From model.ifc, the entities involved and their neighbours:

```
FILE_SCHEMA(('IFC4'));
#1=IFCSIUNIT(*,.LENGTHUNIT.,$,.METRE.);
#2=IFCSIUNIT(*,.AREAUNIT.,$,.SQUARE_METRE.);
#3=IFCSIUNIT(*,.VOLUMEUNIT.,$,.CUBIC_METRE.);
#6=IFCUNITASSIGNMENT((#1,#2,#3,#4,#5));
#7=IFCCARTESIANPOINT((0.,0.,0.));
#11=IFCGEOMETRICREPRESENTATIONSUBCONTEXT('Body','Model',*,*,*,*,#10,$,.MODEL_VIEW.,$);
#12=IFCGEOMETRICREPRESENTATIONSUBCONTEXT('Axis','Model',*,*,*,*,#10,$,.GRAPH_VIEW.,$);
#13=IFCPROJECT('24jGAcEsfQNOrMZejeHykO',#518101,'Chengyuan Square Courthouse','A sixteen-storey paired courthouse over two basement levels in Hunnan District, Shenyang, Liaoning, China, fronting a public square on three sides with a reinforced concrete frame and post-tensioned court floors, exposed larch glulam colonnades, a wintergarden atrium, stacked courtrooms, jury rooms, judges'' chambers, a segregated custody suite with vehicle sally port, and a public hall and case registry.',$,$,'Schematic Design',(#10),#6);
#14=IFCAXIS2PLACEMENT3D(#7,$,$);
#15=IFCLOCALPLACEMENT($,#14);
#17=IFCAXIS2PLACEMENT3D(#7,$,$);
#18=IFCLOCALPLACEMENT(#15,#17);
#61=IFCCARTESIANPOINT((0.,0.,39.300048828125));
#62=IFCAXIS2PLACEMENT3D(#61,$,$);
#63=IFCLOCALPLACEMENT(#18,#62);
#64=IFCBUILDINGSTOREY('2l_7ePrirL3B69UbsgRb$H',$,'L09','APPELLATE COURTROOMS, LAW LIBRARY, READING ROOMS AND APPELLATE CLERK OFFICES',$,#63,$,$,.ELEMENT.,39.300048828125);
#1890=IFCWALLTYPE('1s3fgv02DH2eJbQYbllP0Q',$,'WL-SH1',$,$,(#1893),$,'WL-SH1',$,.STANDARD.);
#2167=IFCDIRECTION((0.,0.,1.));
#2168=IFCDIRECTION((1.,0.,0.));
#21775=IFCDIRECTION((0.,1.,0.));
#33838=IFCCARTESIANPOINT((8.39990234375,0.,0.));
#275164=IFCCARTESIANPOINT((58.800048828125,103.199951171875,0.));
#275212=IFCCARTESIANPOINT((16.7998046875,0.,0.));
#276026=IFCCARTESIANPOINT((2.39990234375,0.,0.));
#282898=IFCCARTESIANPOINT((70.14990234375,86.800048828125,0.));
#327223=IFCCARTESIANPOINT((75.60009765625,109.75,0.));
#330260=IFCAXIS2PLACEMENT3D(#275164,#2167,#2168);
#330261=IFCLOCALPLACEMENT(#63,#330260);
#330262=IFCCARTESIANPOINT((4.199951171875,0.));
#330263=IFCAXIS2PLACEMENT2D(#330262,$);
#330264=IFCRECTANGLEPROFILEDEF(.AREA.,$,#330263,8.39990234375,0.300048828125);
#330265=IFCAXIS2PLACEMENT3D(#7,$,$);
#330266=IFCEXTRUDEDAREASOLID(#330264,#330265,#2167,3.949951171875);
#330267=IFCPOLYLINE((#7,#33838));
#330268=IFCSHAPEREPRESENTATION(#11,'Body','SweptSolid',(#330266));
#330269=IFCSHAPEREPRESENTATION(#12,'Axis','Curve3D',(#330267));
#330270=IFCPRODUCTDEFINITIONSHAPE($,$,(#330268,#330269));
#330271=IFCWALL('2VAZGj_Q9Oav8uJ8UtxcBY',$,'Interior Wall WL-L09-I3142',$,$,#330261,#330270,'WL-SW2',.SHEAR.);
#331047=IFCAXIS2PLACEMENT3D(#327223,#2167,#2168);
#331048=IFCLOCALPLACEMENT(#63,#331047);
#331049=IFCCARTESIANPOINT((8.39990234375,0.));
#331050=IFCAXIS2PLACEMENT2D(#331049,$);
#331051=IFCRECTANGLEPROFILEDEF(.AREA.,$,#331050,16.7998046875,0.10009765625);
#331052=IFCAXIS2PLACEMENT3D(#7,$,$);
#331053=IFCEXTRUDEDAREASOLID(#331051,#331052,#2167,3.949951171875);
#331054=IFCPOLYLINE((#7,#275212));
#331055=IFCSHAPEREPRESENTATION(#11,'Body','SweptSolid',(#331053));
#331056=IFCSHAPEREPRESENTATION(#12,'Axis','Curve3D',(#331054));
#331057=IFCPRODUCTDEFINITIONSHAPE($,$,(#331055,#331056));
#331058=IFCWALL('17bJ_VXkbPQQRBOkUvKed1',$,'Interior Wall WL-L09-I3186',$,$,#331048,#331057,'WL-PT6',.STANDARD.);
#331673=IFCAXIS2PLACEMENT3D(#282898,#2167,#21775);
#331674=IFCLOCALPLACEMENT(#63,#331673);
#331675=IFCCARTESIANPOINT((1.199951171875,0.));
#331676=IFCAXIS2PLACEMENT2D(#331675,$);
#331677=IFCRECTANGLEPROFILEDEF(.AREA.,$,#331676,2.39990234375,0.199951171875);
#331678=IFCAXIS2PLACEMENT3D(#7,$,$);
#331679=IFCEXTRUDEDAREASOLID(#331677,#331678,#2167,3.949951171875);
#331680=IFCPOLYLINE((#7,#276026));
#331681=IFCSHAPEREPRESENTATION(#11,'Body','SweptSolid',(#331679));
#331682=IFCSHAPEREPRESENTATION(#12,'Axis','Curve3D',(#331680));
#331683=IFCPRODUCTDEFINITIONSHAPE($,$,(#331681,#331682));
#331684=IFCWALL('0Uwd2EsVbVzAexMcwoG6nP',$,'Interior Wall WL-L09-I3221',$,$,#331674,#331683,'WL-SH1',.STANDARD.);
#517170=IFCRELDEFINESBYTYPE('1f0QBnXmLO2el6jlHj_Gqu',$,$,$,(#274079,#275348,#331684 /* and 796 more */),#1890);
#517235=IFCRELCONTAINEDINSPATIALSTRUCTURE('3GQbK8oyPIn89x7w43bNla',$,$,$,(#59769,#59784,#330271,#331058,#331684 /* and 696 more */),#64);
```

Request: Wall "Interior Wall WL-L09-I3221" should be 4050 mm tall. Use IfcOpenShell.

```python
import ifcopenshell
import ifcopenshell.geom
import ifcopenshell.util.representation
import ifcopenshell.util.shape

model = ifcopenshell.open("model.ifc")
settings = ifcopenshell.geom.settings()


def volume(element):
    """Net volume in cubic metres, openings subtracted."""
    shape = ifcopenshell.geom.create_shape(settings, element)
    return ifcopenshell.util.shape.get_volume(shape.geometry)


wall = model.by_guid("0Uwd2EsVbVzAexMcwoG6nP")
before = volume(wall)

body = ifcopenshell.util.representation.get_representation(wall, "Model", "Body")
solid = body.Items[0]
old_height = solid.Depth
solid.Depth = 4.05
after = volume(wall)

print(f"height {old_height:g} -> {solid.Depth:g}, volume {before:.3f} -> {after:.3f} m3")

model.write("model_rev.ifc")
```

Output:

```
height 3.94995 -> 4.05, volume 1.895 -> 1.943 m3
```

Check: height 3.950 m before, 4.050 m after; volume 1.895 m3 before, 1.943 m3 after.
